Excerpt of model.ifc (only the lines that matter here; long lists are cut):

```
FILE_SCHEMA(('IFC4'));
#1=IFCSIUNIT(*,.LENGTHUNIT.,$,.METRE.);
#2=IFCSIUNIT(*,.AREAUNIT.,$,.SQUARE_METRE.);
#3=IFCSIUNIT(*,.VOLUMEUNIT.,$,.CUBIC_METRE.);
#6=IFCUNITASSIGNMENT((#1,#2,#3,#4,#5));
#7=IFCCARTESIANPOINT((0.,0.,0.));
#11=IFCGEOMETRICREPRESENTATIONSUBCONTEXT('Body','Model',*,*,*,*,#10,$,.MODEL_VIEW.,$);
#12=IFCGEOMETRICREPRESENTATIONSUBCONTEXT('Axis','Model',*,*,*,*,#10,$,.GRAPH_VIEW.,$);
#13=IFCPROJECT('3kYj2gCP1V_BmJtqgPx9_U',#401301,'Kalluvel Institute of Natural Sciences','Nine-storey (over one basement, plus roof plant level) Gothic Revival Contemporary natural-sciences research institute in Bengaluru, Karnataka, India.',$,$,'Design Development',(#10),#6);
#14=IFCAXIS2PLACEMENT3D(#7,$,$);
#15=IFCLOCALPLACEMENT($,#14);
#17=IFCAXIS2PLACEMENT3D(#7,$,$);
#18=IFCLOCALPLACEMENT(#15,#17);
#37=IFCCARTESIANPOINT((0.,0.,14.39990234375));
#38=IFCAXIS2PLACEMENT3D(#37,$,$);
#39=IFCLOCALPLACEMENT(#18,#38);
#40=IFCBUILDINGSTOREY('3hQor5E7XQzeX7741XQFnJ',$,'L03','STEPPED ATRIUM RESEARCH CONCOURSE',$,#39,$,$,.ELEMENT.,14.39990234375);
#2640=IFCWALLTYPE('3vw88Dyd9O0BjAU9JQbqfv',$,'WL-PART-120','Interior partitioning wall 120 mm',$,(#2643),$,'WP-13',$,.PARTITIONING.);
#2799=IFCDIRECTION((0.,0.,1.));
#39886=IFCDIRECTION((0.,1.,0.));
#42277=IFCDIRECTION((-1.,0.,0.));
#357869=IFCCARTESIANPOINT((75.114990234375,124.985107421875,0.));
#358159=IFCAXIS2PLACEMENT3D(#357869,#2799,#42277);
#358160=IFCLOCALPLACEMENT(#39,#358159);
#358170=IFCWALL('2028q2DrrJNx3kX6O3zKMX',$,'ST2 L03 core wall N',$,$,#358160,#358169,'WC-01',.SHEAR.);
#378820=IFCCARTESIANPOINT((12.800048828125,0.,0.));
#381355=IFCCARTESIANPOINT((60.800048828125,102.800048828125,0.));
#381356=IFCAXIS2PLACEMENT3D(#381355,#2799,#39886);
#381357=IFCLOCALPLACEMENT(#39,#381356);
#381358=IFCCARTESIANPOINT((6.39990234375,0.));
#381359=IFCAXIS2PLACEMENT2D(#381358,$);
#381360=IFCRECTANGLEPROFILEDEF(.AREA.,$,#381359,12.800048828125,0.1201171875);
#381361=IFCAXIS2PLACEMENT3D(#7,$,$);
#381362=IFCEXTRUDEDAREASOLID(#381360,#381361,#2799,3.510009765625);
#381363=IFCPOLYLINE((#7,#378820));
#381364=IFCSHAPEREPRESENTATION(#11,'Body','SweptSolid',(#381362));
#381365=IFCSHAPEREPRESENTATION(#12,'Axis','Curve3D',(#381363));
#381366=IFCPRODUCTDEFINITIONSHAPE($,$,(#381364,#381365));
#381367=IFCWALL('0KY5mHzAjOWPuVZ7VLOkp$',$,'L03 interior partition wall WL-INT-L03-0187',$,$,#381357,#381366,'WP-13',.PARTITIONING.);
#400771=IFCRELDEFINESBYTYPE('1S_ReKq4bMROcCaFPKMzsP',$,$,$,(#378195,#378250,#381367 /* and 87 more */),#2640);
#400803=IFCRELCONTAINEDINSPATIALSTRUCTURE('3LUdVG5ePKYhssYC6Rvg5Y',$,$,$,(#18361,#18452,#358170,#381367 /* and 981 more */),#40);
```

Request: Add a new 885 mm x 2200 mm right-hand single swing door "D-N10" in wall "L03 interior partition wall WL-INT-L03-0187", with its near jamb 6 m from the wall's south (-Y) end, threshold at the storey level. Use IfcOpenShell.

```python
import numpy as np
import ifcopenshell
import ifcopenshell.api.feature
import ifcopenshell.api.geometry
import ifcopenshell.api.root
import ifcopenshell.api.spatial
import ifcopenshell.geom
import ifcopenshell.util.element
import ifcopenshell.util.placement
import ifcopenshell.util.representation
import ifcopenshell.util.shape
import ifcopenshell.util.unit

model = ifcopenshell.open("model.ifc")
unit_scale = ifcopenshell.util.unit.calculate_unit_scale(model)
settings = ifcopenshell.geom.settings()


def volume(element):
    """Net volume in cubic metres, openings subtracted."""
    shape = ifcopenshell.geom.create_shape(settings, element)
    return ifcopenshell.util.shape.get_volume(shape.geometry)


wall = model.by_guid("0KY5mHzAjOWPuVZ7VLOkp$")
storey = ifcopenshell.util.element.get_container(wall, ifc_class="IfcBuildingStorey")
context = ifcopenshell.util.representation.get_context(model, "Model", "Body", "MODEL_VIEW")
before = volume(wall)

width, height, from_end, sill = 0.885, 2.2, 6, 0.0  # metres

# The wall runs along its own X axis, and the end named is its -X end.
wall_shape = ifcopenshell.geom.create_shape(settings, wall)
x, y, z = ifcopenshell.util.shape.get_vertices(wall_shape.geometry).T
start = x.min() + from_end
face, thickness = float(y.min()), float(y.max() - y.min())
wall_matrix = ifcopenshell.util.placement.get_local_placement(wall.ObjectPlacement)
level = ifcopenshell.util.placement.get_local_placement(storey.ObjectPlacement)[2, 3]


def in_wall(x, y):
    """Placement at x, y metres in the wall's axes, at sill height."""
    matrix = wall_matrix.copy()
    matrix[:, 3] = wall_matrix @ np.array([x / unit_scale, y / unit_scale, 0.0, 1.0])
    matrix[2, 3] = level + sill / unit_scale
    return matrix


# Opening: a box that overshoots both wall faces by 50 mm.
opening = ifcopenshell.api.root.create_entity(model, ifc_class="IfcOpeningElement", predefined_type="OPENING")
box = ifcopenshell.api.geometry.add_wall_representation(
    model, context=context, length=width, height=height, thickness=thickness + 0.1
)
ifcopenshell.api.geometry.assign_representation(model, product=opening, representation=box)
ifcopenshell.api.geometry.edit_object_placement(model, product=opening, matrix=in_wall(start, face - 0.05), is_si=False)
ifcopenshell.api.feature.add_feature(model, feature=opening, element=wall)

door = ifcopenshell.api.root.create_entity(model, ifc_class="IfcDoor", name="D-N10", predefined_type="DOOR")
door.OverallWidth, door.OverallHeight = width / unit_scale, height / unit_scale
door.OperationType = "SINGLE_SWING_RIGHT"
body = ifcopenshell.api.geometry.add_door_representation(
    model,
    context=context,
    overall_width=door.OverallWidth,
    overall_height=door.OverallHeight,
    operation_type="SINGLE_SWING_RIGHT",
    lining_properties={"LiningDepth": thickness / unit_scale, "ThresholdDepth": thickness / unit_scale},
)
ifcopenshell.api.geometry.assign_representation(model, product=door, representation=body)
ifcopenshell.api.spatial.assign_container(model, products=[door], relating_structure=storey)
ifcopenshell.api.feature.add_filling(model, opening=opening, element=door)

# The lining spans the wall, so the door starts at the wall face.
ifcopenshell.api.geometry.edit_object_placement(model, product=door, matrix=in_wall(start, face), is_si=False)

after = volume(wall)

print(f"wall volume {before:.3f} -> {after:.3f} m3")

model.write("model_edited.ifc")
```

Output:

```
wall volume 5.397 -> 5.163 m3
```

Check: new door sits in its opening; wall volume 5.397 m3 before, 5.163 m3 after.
